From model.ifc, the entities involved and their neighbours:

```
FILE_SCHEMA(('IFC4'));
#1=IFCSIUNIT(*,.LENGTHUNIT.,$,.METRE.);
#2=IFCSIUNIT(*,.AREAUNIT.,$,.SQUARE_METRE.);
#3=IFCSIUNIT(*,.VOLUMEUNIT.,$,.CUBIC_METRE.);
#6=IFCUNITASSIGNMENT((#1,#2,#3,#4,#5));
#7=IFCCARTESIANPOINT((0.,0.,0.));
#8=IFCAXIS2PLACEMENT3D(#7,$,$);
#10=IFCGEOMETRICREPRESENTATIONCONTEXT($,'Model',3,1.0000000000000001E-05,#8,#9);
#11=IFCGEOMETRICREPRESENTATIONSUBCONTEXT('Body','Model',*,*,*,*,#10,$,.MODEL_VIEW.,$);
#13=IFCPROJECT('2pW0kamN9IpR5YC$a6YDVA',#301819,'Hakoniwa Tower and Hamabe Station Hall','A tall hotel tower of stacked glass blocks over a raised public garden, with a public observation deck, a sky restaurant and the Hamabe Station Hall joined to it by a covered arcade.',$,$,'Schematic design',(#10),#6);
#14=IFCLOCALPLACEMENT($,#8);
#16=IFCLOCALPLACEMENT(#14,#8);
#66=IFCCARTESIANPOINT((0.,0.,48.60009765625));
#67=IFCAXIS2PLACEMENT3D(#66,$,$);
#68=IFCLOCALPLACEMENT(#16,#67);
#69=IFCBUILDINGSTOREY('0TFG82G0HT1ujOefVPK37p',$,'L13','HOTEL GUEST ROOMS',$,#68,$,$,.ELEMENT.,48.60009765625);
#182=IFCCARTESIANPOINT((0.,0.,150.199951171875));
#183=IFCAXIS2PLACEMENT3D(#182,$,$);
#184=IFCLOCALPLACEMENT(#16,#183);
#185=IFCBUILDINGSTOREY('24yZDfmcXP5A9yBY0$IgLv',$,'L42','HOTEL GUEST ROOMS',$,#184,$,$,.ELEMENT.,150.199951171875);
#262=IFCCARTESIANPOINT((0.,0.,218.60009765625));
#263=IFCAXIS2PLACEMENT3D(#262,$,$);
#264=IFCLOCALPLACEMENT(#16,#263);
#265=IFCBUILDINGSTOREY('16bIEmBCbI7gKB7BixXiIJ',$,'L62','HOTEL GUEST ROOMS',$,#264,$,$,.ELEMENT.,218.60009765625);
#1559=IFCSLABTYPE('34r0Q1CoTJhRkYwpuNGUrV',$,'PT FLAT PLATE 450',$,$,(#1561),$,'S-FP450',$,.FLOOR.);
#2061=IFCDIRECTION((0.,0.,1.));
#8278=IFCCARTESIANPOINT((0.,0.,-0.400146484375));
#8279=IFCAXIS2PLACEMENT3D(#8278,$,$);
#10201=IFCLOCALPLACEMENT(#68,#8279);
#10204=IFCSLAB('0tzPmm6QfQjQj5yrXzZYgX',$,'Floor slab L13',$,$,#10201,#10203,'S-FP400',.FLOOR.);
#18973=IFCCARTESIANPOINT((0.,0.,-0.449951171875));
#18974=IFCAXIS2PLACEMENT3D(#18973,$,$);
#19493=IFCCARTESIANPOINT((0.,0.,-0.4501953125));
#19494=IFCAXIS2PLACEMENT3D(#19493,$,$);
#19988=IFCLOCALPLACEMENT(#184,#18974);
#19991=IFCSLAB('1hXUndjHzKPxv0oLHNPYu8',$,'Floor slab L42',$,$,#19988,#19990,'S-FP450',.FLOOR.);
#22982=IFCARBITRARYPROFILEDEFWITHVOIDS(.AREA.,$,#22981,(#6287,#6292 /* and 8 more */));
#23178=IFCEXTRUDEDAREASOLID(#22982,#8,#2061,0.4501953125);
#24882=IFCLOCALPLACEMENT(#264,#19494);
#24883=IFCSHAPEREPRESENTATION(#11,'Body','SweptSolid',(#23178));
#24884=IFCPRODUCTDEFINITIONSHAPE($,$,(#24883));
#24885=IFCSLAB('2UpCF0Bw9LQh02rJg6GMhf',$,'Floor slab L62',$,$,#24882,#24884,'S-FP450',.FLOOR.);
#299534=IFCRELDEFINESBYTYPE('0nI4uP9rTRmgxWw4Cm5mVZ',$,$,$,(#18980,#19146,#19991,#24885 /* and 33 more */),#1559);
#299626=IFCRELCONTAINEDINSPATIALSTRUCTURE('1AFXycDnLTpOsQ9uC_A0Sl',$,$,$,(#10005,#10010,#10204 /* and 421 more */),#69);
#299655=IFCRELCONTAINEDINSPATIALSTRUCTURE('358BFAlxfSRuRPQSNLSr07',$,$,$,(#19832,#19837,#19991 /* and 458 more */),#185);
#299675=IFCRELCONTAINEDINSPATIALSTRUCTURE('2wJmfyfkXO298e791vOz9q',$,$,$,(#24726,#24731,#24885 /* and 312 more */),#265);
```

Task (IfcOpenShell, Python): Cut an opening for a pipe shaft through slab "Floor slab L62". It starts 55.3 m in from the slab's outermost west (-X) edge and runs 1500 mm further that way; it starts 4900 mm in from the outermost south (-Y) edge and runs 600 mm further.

```python
import numpy as np
import ifcopenshell
import ifcopenshell.api.feature
import ifcopenshell.api.geometry
import ifcopenshell.api.root
import ifcopenshell.geom
import ifcopenshell.util.placement
import ifcopenshell.util.representation
import ifcopenshell.util.shape
import ifcopenshell.util.unit

model = ifcopenshell.open("model.ifc")
unit_scale = ifcopenshell.util.unit.calculate_unit_scale(model)
settings = ifcopenshell.geom.settings()


def volume(element):
    """Net volume in cubic metres, openings subtracted."""
    shape = ifcopenshell.geom.create_shape(settings, element)
    return ifcopenshell.util.shape.get_volume(shape.geometry)


slab = model.by_id(24885)
before = volume(slab)

# Extent in the slab's own axes, in metres. The edges named are its -X and -Y sides.
slab_shape = ifcopenshell.geom.create_shape(settings, slab)
vertices = ifcopenshell.util.shape.get_vertices(slab_shape.geometry)
x_min, y_min, bottom = vertices.min(axis=0)
top = vertices[:, 2].max()

opening = ifcopenshell.api.root.create_entity(model, ifc_class="IfcOpeningElement", name="Pipe shaft opening", predefined_type="OPENING")
context = ifcopenshell.util.representation.get_context(model, "Model", "Body", "MODEL_VIEW")
width, depth = 1.5, 0.6
outline = [(0.0, 0.0), (width, 0.0), (width, depth), (0.0, depth), (0.0, 0.0)]
# Overshoot both faces by 50 mm so the cut is clean.
shape = ifcopenshell.api.geometry.add_slab_representation(
    model, context=context, depth=top - bottom + 0.1, polyline=outline
)
ifcopenshell.api.geometry.assign_representation(model, product=opening, representation=shape)

matrix = ifcopenshell.util.placement.get_local_placement(slab.ObjectPlacement)
matrix[:, 3] = matrix @ np.append(np.array([x_min + 55.3, y_min + 4.9, bottom - 0.05]) / unit_scale, 1.0)
ifcopenshell.api.geometry.edit_object_placement(model, product=opening, matrix=matrix, is_si=False)
ifcopenshell.api.feature.add_feature(model, feature=opening, element=slab)

after = volume(slab)

print(f"slab volume {before:.3f} -> {after:.3f} m3")

model.write("model_updated.ifc")
```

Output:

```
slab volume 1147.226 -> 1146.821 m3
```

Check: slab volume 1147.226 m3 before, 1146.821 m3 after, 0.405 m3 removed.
